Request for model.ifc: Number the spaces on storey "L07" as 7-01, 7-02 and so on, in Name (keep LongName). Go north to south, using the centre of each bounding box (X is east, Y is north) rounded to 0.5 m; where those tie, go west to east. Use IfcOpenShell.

First a look at what the model holds.

```python
import ifcopenshell
import ifcopenshell.util.element
import ifcopenshell.util.placement

model = ifcopenshell.open("model.ifc")
print(model.schema)
storey = next(s for s in model.by_type("IfcBuildingStorey") if s.Name == "L07")
spaces = [e for e in ifcopenshell.util.element.get_decomposition(storey) if e.is_a("IfcSpace")]
for e in sorted(spaces, key=lambda e: e.id()):
    origin = ifcopenshell.util.placement.get_local_placement(e.ObjectPlacement)[:3, 3]
    print(e.id(), e.Name, e.LongName, origin.round(2) + 0.0, sep=" | ")
```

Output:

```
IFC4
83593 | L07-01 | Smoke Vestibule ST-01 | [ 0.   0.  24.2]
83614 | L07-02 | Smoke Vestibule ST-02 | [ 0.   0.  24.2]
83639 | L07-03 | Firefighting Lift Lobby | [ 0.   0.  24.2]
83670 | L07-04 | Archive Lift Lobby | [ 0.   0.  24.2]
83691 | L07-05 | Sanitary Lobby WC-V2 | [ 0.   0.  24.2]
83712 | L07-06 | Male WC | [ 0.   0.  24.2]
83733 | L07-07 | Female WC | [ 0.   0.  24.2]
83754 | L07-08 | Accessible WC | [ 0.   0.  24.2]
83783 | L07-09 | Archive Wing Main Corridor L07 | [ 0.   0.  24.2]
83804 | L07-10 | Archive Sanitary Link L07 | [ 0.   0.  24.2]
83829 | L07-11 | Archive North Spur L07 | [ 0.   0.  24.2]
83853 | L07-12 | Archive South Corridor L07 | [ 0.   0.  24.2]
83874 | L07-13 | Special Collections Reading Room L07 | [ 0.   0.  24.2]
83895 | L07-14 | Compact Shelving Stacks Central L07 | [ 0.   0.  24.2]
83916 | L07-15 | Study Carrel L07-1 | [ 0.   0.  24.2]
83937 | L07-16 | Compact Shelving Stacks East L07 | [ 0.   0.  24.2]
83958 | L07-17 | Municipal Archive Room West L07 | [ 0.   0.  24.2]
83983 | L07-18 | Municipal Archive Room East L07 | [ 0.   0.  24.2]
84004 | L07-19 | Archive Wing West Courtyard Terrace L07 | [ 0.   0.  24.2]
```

```python
import ifcopenshell
import ifcopenshell.geom
import ifcopenshell.util.element
import ifcopenshell.util.shape

model = ifcopenshell.open("model.ifc")
settings = ifcopenshell.geom.settings()
settings.set("use-world-coords", True)


def centre(element):
    shape = ifcopenshell.geom.create_shape(settings, element)
    return ifcopenshell.util.shape.get_bbox_centroid(shape.geometry)


storey = next(s for s in model.by_type("IfcBuildingStorey") if s.Name == "L07")
spaces = [e for e in ifcopenshell.util.element.get_decomposition(storey) if e.is_a("IfcSpace")]

# Insertion points can sit at a corner or the storey origin, so sort by the geometry (in metres).
centres = {e: centre(e) for e in spaces}
spaces.sort(key=lambda e: (-round(centres[e][1] / 0.5), centres[e][0]))

for i, e in enumerate(spaces, start=1):
    number = f"7-{i:02d}"
    e.Name = number
    print(e.id(), number)

model.write("model_v2.ifc")
```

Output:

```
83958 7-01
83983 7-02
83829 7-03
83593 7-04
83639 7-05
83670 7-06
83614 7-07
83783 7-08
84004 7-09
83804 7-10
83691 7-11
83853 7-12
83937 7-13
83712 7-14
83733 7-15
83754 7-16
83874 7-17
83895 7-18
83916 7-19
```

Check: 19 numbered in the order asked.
